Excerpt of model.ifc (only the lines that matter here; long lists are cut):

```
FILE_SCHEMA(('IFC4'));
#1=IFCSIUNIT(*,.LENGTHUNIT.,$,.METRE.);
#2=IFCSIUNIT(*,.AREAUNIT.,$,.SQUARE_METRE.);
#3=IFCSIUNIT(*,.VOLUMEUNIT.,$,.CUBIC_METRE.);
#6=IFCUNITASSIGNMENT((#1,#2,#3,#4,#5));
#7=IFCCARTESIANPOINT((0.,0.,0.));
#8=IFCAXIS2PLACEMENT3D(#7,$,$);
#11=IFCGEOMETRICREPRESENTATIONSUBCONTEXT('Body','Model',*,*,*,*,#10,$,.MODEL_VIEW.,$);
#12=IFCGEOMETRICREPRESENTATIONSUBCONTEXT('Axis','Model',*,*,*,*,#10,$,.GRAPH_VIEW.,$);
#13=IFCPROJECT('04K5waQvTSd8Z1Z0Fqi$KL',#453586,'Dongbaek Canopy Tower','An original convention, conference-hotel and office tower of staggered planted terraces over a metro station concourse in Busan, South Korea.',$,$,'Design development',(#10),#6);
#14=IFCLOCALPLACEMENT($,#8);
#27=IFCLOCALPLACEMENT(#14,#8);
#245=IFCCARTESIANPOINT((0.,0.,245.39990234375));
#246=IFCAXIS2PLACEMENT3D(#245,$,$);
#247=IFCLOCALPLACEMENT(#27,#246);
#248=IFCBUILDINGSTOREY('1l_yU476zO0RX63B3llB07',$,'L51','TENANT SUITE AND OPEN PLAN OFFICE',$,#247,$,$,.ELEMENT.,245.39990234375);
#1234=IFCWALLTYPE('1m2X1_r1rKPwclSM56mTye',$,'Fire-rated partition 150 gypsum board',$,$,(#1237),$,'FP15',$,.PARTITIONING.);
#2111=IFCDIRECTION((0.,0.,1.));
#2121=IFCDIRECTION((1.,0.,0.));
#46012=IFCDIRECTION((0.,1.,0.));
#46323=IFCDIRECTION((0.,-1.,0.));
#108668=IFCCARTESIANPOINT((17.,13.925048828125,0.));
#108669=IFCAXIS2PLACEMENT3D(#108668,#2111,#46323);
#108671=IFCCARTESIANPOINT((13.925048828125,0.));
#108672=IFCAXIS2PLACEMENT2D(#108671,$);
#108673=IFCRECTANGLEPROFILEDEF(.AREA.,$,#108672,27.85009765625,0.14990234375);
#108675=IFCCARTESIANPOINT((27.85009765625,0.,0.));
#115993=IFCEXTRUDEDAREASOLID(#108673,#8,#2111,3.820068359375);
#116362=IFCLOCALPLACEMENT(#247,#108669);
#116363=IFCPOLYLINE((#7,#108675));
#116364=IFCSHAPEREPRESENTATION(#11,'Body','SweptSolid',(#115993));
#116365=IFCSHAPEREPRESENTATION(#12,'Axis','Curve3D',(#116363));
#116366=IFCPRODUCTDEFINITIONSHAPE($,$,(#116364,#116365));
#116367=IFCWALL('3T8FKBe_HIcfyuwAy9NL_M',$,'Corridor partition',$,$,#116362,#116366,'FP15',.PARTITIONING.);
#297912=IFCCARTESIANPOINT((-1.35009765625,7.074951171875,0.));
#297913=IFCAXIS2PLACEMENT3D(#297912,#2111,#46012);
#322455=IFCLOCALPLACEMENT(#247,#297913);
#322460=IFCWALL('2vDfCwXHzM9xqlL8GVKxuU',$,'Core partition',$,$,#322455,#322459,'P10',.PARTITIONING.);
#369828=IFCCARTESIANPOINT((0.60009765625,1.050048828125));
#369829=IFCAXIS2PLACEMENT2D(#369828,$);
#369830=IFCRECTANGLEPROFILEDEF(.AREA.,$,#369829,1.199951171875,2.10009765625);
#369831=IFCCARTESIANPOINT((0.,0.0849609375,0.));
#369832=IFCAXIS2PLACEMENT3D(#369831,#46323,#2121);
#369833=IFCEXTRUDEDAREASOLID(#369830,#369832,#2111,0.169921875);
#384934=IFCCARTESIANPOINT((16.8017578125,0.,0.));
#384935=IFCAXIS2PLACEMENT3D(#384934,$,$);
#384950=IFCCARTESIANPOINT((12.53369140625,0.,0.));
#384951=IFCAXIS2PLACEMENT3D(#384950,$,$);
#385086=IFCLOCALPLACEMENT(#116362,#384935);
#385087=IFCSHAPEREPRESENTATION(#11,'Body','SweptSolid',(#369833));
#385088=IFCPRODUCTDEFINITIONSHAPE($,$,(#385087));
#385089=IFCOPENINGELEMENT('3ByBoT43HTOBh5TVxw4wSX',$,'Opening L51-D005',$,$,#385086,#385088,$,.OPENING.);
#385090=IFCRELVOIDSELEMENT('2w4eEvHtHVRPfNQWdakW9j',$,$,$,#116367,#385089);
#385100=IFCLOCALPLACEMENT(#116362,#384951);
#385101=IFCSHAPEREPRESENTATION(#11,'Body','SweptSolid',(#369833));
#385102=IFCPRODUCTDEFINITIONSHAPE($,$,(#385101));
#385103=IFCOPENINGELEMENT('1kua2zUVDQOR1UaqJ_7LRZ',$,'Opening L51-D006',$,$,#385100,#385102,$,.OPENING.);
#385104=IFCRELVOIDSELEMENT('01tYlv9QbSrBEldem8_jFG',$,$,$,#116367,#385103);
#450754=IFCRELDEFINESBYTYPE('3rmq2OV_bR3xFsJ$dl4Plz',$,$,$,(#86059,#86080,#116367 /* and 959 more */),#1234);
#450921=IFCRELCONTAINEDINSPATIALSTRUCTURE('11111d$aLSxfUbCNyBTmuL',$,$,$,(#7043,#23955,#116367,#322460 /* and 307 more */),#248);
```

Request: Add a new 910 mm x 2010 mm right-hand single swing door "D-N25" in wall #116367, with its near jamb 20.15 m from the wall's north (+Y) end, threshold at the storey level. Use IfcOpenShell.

```python
import numpy as np
import ifcopenshell
import ifcopenshell.api.feature
import ifcopenshell.api.geometry
import ifcopenshell.api.root
import ifcopenshell.api.spatial
import ifcopenshell.geom
import ifcopenshell.util.element
import ifcopenshell.util.placement
import ifcopenshell.util.representation
import ifcopenshell.util.shape
import ifcopenshell.util.unit

model = ifcopenshell.open("model.ifc")
unit_scale = ifcopenshell.util.unit.calculate_unit_scale(model)
settings = ifcopenshell.geom.settings()


def volume(element):
    """Net volume in cubic metres, openings subtracted."""
    shape = ifcopenshell.geom.create_shape(settings, element)
    return ifcopenshell.util.shape.get_volume(shape.geometry)


wall = model.by_guid("3T8FKBe_HIcfyuwAy9NL_M")
storey = ifcopenshell.util.element.get_container(wall, ifc_class="IfcBuildingStorey")
context = ifcopenshell.util.representation.get_context(model, "Model", "Body", "MODEL_VIEW")
before = volume(wall)

width, height, from_end, sill = 0.91, 2.01, 20.15, 0.0  # metres

# The wall runs along its own X axis, and the end named is its -X end.
wall_shape = ifcopenshell.geom.create_shape(settings, wall)
x, y, z = ifcopenshell.util.shape.get_vertices(wall_shape.geometry).T
start = x.min() + from_end
face, thickness = float(y.min()), float(y.max() - y.min())
wall_matrix = ifcopenshell.util.placement.get_local_placement(wall.ObjectPlacement)
level = ifcopenshell.util.placement.get_local_placement(storey.ObjectPlacement)[2, 3]


def in_wall(x, y):
    """Placement at x, y metres in the wall's axes, at sill height."""
    matrix = wall_matrix.copy()
    matrix[:, 3] = wall_matrix @ np.array([x / unit_scale, y / unit_scale, 0.0, 1.0])
    matrix[2, 3] = level + sill / unit_scale
    return matrix


# Opening: a box that overshoots both wall faces by 50 mm.
opening = ifcopenshell.api.root.create_entity(model, ifc_class="IfcOpeningElement", predefined_type="OPENING")
box = ifcopenshell.api.geometry.add_wall_representation(
    model, context=context, length=width, height=height, thickness=thickness + 0.1
)
ifcopenshell.api.geometry.assign_representation(model, product=opening, representation=box)
ifcopenshell.api.geometry.edit_object_placement(model, product=opening, matrix=in_wall(start, face - 0.05), is_si=False)
ifcopenshell.api.feature.add_feature(model, feature=opening, element=wall)

door = ifcopenshell.api.root.create_entity(model, ifc_class="IfcDoor", name="D-N25", predefined_type="DOOR")
door.OverallWidth, door.OverallHeight = width / unit_scale, height / unit_scale
door.OperationType = "SINGLE_SWING_RIGHT"
body = ifcopenshell.api.geometry.add_door_representation(
    model,
    context=context,
    overall_width=door.OverallWidth,
    overall_height=door.OverallHeight,
    operation_type="SINGLE_SWING_RIGHT",
    lining_properties={"LiningDepth": thickness / unit_scale, "ThresholdDepth": thickness / unit_scale},
)
ifcopenshell.api.geometry.assign_representation(model, product=door, representation=body)
ifcopenshell.api.spatial.assign_container(model, products=[door], relating_structure=storey)
ifcopenshell.api.feature.add_filling(model, opening=opening, element=door)

# The lining spans the wall, so the door starts at the wall face.
ifcopenshell.api.geometry.edit_object_placement(model, product=door, matrix=in_wall(start, face), is_si=False)

after = volume(wall)

print(f"wall volume {before:.3f} -> {after:.3f} m3")

model.write("model_updated.ifc")
```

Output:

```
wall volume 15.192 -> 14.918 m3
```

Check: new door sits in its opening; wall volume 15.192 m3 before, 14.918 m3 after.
